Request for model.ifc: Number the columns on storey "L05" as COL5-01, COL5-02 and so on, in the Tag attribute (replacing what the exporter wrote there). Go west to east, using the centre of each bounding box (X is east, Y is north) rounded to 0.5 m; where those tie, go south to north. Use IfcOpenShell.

First a look at what the model holds.

```python
import ifcopenshell
import ifcopenshell.util.element
import ifcopenshell.util.placement

model = ifcopenshell.open("model.ifc")
print(model.schema)
storey = next(s for s in model.by_type("IfcBuildingStorey") if s.Name == "L05")
columns = [e for e in ifcopenshell.util.element.get_decomposition(storey) if e.is_a("IfcColumn")]
for e in sorted(columns, key=lambda e: e.id()):
    origin = ifcopenshell.util.placement.get_local_placement(e.ObjectPlacement)[:3, 3]
    print(e.id(), e.Tag, e.Name, origin.round(2) + 0.0, sep=" | ")
```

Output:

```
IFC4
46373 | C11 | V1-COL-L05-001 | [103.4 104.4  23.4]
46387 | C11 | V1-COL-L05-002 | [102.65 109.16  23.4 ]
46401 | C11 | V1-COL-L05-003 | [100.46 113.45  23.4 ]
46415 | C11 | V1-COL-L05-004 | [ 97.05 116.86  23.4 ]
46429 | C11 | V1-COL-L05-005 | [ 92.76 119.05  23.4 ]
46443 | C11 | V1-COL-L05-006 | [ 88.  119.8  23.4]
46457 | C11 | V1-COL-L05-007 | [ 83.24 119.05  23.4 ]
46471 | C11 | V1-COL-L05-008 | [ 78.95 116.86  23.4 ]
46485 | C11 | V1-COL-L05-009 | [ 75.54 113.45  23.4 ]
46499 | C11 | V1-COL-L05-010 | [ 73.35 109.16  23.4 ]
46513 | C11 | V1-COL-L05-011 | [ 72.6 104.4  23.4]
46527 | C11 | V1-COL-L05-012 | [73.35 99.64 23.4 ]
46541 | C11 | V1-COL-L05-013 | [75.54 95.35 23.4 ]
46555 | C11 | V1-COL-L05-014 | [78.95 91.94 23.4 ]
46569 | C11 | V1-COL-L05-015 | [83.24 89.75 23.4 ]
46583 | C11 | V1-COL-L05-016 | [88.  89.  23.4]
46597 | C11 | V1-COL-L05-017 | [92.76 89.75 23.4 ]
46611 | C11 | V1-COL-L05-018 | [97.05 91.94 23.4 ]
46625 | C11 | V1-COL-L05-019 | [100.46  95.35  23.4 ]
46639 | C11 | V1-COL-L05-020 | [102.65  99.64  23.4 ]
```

```python
import ifcopenshell
import ifcopenshell.geom
import ifcopenshell.util.element
import ifcopenshell.util.shape

model = ifcopenshell.open("model.ifc")
settings = ifcopenshell.geom.settings()
settings.set("use-world-coords", True)


def centre(element):
    shape = ifcopenshell.geom.create_shape(settings, element)
    return ifcopenshell.util.shape.get_bbox_centroid(shape.geometry)


storey = next(s for s in model.by_type("IfcBuildingStorey") if s.Name == "L05")
columns = [e for e in ifcopenshell.util.element.get_decomposition(storey) if e.is_a("IfcColumn")]

# Insertion points can sit at a corner or the storey origin, so sort by the geometry (in metres).
centres = {e: centre(e) for e in columns}
columns.sort(key=lambda e: (round(centres[e][0] / 0.5), centres[e][1]))

for i, e in enumerate(columns, start=1):
    number = f"COL5-{i:02d}"
    e.Tag = number
    print(e.id(), number)

model.write("model_v2.ifc")
```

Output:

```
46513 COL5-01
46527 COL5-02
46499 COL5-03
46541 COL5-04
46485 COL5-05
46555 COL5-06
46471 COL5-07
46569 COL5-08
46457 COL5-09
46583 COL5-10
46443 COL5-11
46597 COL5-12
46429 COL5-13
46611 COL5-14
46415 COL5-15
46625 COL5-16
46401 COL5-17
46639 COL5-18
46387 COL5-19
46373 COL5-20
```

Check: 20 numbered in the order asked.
